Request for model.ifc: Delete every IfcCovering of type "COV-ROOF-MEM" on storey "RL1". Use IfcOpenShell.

First a look at what the model holds.

```python
import ifcopenshell
import ifcopenshell.util.element

model = ifcopenshell.open("model.ifc")
print(model.schema)
storey = next(s for s in model.by_type("IfcBuildingStorey") if s.Name == "RL1")
coverings = [e for e in ifcopenshell.util.element.get_decomposition(storey) if e.is_a("IfcCovering")]
seen = {}
for e in coverings:
    element_type = ifcopenshell.util.element.get_type(e)
    name = element_type.Name if element_type not in (None, e) else None
    seen[name] = seen.get(name, 0) + 1
for name, count in sorted(seen.items(), key=str):
    print(count, "x", name)
```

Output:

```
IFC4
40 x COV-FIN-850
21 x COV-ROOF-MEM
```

```python
import ifcopenshell
import ifcopenshell.api.root
import ifcopenshell.util.element

model = ifcopenshell.open("model.ifc")

storey = next(s for s in model.by_type("IfcBuildingStorey") if s.Name == "RL1")
coverings = [e for e in ifcopenshell.util.element.get_decomposition(storey) if e.is_a("IfcCovering")]
targets = [e for e in coverings if (t := ifcopenshell.util.element.get_type(e)) not in (None, e) and t.Name == "COV-ROOF-MEM"]

for e in targets:
    ifcopenshell.api.root.remove_product(model, product=e)
print(len(targets), "removed")

model.write("model_updated.ifc")
```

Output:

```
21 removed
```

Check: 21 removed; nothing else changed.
